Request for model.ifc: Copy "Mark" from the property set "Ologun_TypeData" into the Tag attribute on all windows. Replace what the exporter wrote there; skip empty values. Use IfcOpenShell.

First a look at what the model holds.

```python
import ifcopenshell
import ifcopenshell.util.element

model = ifcopenshell.open("model.ifc")
print(model.schema)
windows = model.by_type("IfcWindow")
print(len(windows), "windows")
for e in windows[:8]:
    source = ifcopenshell.util.element.get_pset(e, "Ologun_TypeData", "Mark")
    target = e.Tag
    print(e.id(), repr(source), repr(target), sep=" | ")
```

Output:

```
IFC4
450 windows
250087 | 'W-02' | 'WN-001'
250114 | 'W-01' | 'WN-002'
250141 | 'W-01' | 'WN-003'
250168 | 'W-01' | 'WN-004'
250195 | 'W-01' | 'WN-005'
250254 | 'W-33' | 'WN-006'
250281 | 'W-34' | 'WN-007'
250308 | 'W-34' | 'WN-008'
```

```python
import ifcopenshell
import ifcopenshell.util.element

model = ifcopenshell.open("model.ifc")

count = 0
for e in model.by_type("IfcWindow"):
    value = ifcopenshell.util.element.get_pset(e, "Ologun_TypeData", "Mark")
    current = e.Tag
    if not value or not value.strip() or current == value:
        continue
    e.Tag = value
    count += 1

print(count, "windows updated")

model.write("model_rev.ifc")
```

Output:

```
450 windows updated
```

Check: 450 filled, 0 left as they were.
